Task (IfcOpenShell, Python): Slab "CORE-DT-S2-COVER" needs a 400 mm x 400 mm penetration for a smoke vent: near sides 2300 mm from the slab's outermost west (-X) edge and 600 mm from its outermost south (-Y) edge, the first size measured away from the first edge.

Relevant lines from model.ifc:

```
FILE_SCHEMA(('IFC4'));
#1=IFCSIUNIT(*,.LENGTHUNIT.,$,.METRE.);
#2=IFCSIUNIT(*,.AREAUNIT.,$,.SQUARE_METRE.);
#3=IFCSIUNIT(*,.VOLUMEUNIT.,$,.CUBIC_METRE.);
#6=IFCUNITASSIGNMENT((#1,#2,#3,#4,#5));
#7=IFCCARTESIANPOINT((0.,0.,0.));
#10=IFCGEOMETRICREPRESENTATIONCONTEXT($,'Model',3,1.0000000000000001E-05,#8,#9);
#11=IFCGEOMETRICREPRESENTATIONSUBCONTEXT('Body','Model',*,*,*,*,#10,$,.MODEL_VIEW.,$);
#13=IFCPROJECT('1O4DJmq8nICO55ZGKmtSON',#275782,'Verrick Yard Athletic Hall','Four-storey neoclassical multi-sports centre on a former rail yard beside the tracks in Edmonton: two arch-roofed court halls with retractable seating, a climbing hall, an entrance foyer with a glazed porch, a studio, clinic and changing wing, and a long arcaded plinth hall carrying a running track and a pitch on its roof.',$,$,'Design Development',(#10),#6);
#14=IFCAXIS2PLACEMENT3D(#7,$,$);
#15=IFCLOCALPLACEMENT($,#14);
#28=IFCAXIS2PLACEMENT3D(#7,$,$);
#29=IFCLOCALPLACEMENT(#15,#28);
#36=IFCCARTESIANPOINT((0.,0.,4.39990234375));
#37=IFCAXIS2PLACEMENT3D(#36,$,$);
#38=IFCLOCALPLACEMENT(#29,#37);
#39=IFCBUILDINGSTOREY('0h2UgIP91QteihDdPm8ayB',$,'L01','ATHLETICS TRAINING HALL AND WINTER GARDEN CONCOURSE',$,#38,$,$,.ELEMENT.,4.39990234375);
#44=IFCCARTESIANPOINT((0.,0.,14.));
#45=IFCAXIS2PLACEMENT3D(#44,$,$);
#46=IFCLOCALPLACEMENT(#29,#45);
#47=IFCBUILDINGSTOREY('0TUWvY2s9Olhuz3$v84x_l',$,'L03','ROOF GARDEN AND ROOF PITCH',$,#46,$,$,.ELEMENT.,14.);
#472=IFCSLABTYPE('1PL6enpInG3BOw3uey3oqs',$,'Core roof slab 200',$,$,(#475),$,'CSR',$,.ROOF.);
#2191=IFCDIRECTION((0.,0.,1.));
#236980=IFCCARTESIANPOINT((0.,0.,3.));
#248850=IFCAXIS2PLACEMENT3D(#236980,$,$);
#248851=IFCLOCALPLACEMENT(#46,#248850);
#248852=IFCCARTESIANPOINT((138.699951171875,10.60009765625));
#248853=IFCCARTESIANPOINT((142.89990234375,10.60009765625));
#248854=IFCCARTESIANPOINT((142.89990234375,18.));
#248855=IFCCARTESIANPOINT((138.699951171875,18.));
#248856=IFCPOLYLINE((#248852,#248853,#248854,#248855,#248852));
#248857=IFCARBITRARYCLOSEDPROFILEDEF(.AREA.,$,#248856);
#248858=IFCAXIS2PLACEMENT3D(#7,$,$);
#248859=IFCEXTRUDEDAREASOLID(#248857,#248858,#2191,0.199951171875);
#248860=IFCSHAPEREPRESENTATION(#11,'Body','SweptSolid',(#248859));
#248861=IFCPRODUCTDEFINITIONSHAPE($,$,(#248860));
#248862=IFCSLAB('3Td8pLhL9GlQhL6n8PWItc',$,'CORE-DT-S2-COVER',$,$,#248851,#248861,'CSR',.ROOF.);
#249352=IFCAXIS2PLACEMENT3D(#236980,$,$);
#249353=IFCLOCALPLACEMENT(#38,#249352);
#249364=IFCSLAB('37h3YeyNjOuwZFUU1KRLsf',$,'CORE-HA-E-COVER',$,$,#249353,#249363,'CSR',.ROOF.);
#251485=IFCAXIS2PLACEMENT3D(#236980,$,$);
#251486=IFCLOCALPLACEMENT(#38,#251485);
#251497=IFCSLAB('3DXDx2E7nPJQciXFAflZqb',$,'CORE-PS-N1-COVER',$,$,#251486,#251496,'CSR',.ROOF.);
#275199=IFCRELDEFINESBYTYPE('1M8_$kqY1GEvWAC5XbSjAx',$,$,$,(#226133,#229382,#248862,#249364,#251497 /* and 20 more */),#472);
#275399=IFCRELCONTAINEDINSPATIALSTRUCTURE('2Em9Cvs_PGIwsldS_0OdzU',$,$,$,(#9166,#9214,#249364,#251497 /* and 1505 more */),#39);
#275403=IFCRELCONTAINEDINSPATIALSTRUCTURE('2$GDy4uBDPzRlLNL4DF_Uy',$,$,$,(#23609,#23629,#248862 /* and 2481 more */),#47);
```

```python
import numpy as np
import ifcopenshell
import ifcopenshell.api.feature
import ifcopenshell.api.geometry
import ifcopenshell.api.root
import ifcopenshell.geom
import ifcopenshell.util.placement
import ifcopenshell.util.representation
import ifcopenshell.util.shape
import ifcopenshell.util.unit

model = ifcopenshell.open("model.ifc")
unit_scale = ifcopenshell.util.unit.calculate_unit_scale(model)
settings = ifcopenshell.geom.settings()


def volume(element):
    """Net volume in cubic metres, openings subtracted."""
    shape = ifcopenshell.geom.create_shape(settings, element)
    return ifcopenshell.util.shape.get_volume(shape.geometry)


slab = model.by_id(248862)
before = volume(slab)

# Extent in the slab's own axes, in metres. The edges named are its -X and -Y sides.
slab_shape = ifcopenshell.geom.create_shape(settings, slab)
vertices = ifcopenshell.util.shape.get_vertices(slab_shape.geometry)
x_min, y_min, bottom = vertices.min(axis=0)
top = vertices[:, 2].max()

opening = ifcopenshell.api.root.create_entity(model, ifc_class="IfcOpeningElement", name="Smoke vent opening", predefined_type="OPENING")
context = ifcopenshell.util.representation.get_context(model, "Model", "Body", "MODEL_VIEW")
width, depth = 0.4, 0.4
outline = [(0.0, 0.0), (width, 0.0), (width, depth), (0.0, depth), (0.0, 0.0)]
# Overshoot both faces by 50 mm so the cut is clean.
shape = ifcopenshell.api.geometry.add_slab_representation(
    model, context=context, depth=top - bottom + 0.1, polyline=outline
)
ifcopenshell.api.geometry.assign_representation(model, product=opening, representation=shape)

matrix = ifcopenshell.util.placement.get_local_placement(slab.ObjectPlacement)
matrix[:, 3] = matrix @ np.append(np.array([x_min + 2.3, y_min + 0.6, bottom - 0.05]) / unit_scale, 1.0)
ifcopenshell.api.geometry.edit_object_placement(model, product=opening, matrix=matrix, is_si=False)
ifcopenshell.api.feature.add_feature(model, feature=opening, element=slab)

after = volume(slab)

print(f"slab volume {before:.3f} -> {after:.3f} m3")

model.write("model-out.ifc")
```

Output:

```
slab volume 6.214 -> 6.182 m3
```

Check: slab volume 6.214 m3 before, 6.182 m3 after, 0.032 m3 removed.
